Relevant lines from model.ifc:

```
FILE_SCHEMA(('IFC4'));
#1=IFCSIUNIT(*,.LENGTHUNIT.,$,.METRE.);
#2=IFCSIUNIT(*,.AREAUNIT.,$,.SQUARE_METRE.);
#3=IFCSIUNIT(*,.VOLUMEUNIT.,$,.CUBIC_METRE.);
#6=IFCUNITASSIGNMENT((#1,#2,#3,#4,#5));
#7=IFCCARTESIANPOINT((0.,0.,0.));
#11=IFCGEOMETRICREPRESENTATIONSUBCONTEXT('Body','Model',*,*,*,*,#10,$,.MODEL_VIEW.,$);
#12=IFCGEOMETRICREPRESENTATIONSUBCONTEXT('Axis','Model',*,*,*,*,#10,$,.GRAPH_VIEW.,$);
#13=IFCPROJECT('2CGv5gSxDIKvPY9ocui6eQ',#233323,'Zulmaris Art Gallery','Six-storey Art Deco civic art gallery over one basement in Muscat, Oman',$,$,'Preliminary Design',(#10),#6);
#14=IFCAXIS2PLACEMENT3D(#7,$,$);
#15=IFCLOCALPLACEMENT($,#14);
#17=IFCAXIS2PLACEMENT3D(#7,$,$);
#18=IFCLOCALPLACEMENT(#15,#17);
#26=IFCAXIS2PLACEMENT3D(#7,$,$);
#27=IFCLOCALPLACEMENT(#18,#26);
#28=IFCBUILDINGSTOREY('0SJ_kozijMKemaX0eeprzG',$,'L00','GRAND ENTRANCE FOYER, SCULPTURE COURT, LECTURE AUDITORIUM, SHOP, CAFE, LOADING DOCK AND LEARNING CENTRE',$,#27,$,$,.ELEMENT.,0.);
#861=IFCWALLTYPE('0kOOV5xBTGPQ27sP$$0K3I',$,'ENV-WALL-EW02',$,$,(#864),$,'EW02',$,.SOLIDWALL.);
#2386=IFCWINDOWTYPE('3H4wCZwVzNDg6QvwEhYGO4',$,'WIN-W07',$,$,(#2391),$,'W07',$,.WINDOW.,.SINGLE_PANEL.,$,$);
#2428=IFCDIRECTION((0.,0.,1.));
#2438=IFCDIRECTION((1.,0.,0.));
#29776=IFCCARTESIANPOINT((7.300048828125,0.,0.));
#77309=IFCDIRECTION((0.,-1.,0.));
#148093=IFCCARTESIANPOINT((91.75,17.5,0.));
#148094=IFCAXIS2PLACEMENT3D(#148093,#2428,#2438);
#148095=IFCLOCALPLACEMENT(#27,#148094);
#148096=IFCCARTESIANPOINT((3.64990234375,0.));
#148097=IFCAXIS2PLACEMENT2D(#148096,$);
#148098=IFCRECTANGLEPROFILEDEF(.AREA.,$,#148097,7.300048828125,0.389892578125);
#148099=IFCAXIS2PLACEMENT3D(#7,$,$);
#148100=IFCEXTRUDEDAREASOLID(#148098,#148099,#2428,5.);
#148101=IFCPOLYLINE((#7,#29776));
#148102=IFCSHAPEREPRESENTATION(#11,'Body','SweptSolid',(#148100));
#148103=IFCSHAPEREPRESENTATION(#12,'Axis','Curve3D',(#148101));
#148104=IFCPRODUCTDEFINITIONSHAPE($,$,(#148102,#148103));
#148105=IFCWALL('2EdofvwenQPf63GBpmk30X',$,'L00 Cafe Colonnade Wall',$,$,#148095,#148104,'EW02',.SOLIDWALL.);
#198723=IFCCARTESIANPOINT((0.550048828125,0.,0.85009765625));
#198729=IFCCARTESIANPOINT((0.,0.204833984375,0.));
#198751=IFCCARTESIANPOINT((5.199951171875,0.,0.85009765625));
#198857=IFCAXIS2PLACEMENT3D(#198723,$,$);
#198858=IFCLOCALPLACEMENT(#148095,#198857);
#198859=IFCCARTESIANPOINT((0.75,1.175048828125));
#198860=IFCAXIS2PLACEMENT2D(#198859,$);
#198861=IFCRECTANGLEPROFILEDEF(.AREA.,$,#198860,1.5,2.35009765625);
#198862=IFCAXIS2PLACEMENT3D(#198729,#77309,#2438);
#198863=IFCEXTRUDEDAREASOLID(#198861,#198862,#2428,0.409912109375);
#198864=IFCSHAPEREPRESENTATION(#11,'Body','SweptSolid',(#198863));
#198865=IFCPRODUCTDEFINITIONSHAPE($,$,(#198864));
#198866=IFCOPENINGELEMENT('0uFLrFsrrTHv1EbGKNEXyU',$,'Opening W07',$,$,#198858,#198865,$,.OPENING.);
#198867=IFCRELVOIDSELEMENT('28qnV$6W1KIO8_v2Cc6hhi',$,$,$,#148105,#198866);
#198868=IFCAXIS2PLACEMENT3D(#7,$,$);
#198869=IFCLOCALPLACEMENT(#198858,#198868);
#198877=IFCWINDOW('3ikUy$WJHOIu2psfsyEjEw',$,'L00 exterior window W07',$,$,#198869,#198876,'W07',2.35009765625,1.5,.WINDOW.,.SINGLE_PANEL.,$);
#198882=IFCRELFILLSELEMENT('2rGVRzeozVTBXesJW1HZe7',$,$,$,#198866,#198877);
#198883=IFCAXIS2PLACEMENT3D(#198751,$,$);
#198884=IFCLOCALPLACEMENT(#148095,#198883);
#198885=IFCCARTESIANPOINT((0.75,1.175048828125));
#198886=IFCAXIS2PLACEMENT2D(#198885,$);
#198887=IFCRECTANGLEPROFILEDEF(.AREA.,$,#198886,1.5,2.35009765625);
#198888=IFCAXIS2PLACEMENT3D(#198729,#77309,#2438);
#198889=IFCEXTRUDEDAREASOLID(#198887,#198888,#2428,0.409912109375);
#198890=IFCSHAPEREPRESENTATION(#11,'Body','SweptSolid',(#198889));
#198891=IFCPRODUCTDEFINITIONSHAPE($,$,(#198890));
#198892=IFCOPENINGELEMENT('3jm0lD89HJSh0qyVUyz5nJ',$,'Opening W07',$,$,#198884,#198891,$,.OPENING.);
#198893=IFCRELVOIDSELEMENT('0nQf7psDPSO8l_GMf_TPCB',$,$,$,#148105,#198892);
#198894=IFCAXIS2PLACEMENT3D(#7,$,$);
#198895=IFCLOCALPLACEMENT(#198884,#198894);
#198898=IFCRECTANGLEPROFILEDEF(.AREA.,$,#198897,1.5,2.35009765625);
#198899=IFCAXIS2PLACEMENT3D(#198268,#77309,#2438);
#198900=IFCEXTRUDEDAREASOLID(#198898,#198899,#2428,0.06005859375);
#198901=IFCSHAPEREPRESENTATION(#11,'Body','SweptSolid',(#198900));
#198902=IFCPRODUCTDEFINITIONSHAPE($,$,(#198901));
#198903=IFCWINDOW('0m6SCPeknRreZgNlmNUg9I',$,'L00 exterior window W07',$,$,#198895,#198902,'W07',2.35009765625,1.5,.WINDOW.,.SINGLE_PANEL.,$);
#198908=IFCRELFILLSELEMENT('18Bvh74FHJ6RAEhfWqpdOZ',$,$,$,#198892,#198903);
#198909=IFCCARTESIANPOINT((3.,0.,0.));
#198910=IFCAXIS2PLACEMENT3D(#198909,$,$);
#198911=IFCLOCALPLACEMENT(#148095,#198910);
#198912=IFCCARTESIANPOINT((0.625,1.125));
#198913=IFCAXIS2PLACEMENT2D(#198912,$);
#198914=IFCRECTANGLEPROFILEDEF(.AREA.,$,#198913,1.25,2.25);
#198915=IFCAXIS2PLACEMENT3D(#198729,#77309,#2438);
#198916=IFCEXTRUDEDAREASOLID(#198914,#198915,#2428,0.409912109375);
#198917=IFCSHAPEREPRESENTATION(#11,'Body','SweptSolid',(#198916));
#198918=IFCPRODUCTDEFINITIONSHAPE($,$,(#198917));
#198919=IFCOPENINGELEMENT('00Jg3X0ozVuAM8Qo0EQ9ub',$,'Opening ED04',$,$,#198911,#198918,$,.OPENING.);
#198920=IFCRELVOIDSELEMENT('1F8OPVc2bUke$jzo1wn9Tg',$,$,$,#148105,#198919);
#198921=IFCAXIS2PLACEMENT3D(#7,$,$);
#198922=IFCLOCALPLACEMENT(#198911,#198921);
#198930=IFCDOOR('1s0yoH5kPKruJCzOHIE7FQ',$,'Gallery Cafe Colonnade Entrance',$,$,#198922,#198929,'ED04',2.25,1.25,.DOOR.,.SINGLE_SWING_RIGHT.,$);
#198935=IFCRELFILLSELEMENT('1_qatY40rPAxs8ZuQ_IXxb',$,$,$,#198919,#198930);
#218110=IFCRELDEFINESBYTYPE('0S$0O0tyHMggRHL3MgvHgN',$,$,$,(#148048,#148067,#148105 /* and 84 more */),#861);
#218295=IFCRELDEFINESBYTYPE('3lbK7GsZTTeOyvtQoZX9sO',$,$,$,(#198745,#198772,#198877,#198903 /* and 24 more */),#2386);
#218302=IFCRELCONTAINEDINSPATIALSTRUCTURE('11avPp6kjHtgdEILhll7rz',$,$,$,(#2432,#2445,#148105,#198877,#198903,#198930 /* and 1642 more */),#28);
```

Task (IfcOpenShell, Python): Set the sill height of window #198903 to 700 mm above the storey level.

```python
import numpy as np
import ifcopenshell
import ifcopenshell.api.geometry
import ifcopenshell.geom
import ifcopenshell.util.element
import ifcopenshell.util.placement
import ifcopenshell.util.shape
import ifcopenshell.util.unit

model = ifcopenshell.open("model.ifc")
unit_scale = ifcopenshell.util.unit.calculate_unit_scale(model)

window = model.by_guid("0m6SCPeknRreZgNlmNUg9I")
opening = window.FillsVoids[0].RelatingOpeningElement
storey = ifcopenshell.util.element.get_container(window, ifc_class="IfcBuildingStorey")
level = ifcopenshell.util.placement.get_local_placement(storey.ObjectPlacement)[2, 3]

# The opening's origin need not be at the sill, so measure its lowest point.
shape = ifcopenshell.geom.create_shape(ifcopenshell.geom.settings(), opening)
bottom = ifcopenshell.util.shape.get_shape_bottom_elevation(shape, shape.geometry) / unit_scale
dz = level + 0.7 / unit_scale - bottom

shift = np.array([0.0, 0.0, dz])
# The window is placed relative to its opening, so it follows when the opening moves.
matrix = ifcopenshell.util.placement.get_local_placement(opening.ObjectPlacement)
matrix[:3, 3] += shift
ifcopenshell.api.geometry.edit_object_placement(
    model, product=opening, matrix=matrix, is_si=False, should_transform_children=True
)

print(f"moved by {dz * unit_scale:+.3f} m")

model.write("model_updated.ifc")
```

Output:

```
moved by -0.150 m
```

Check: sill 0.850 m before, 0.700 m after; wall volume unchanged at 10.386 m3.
